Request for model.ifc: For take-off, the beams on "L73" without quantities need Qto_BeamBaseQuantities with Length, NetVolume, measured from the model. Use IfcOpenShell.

First a look at what the model holds.

```python
import ifcopenshell
import ifcopenshell.util.element
import ifcopenshell.util.unit

model = ifcopenshell.open("model.ifc")
print(model.schema)
for unit_type in ("LENGTHUNIT", "AREAUNIT", "VOLUMEUNIT"):
    print(unit_type, ifcopenshell.util.unit.calculate_unit_scale(model, unit_type))
storey = next(s for s in model.by_type("IfcBuildingStorey") if s.Name == "L73")
beams = [e for e in ifcopenshell.util.element.get_decomposition(storey) if e.is_a("IfcBeam")]
for e in sorted(beams, key=lambda e: e.id()):
    print(e.id(), e.is_a(), e.Name, list(ifcopenshell.util.element.get_psets(e, qtos_only=True)), sep=" | ")
```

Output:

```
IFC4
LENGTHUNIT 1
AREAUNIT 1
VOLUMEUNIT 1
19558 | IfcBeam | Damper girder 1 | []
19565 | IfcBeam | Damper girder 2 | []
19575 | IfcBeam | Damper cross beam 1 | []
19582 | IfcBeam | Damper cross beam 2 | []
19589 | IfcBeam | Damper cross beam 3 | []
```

```python
import ifcopenshell
import ifcopenshell.api.pset
import ifcopenshell.geom
import ifcopenshell.util.element
import ifcopenshell.util.shape
import ifcopenshell.util.unit

model = ifcopenshell.open("model.ifc")
unit_scale = ifcopenshell.util.unit.calculate_unit_scale(model)
volume_scale = ifcopenshell.util.unit.calculate_unit_scale(model, "VOLUMEUNIT")
settings = ifcopenshell.geom.settings()

storey = next(s for s in model.by_type("IfcBuildingStorey") if s.Name == "L73")
beams = [e for e in ifcopenshell.util.element.get_decomposition(storey) if e.is_a("IfcBeam")]

for e in sorted(beams, key=lambda e: e.id()):
    if ifcopenshell.util.element.get_psets(e, qtos_only=True, should_inherit=False):
        continue
    # Geometry comes back in metres, in the element's own axes.
    shape = ifcopenshell.geom.create_shape(settings, e)
    values = {
        "Length": ifcopenshell.util.shape.get_max_xyz(shape.geometry) / unit_scale,
        "NetVolume": ifcopenshell.util.shape.get_volume(shape.geometry) / volume_scale,
    }
    qto = ifcopenshell.api.pset.add_qto(model, product=e, name="Qto_BeamBaseQuantities")
    ifcopenshell.api.pset.edit_qto(model, qto=qto, properties=values)
    print(e.id(), {k: round(v, 3) for k, v in values.items()})

model.write("model_updated.ifc")
```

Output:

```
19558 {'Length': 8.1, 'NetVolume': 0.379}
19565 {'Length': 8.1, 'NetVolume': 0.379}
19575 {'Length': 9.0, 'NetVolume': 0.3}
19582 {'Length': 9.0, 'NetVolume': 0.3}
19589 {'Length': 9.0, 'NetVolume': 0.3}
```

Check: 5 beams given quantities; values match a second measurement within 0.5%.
